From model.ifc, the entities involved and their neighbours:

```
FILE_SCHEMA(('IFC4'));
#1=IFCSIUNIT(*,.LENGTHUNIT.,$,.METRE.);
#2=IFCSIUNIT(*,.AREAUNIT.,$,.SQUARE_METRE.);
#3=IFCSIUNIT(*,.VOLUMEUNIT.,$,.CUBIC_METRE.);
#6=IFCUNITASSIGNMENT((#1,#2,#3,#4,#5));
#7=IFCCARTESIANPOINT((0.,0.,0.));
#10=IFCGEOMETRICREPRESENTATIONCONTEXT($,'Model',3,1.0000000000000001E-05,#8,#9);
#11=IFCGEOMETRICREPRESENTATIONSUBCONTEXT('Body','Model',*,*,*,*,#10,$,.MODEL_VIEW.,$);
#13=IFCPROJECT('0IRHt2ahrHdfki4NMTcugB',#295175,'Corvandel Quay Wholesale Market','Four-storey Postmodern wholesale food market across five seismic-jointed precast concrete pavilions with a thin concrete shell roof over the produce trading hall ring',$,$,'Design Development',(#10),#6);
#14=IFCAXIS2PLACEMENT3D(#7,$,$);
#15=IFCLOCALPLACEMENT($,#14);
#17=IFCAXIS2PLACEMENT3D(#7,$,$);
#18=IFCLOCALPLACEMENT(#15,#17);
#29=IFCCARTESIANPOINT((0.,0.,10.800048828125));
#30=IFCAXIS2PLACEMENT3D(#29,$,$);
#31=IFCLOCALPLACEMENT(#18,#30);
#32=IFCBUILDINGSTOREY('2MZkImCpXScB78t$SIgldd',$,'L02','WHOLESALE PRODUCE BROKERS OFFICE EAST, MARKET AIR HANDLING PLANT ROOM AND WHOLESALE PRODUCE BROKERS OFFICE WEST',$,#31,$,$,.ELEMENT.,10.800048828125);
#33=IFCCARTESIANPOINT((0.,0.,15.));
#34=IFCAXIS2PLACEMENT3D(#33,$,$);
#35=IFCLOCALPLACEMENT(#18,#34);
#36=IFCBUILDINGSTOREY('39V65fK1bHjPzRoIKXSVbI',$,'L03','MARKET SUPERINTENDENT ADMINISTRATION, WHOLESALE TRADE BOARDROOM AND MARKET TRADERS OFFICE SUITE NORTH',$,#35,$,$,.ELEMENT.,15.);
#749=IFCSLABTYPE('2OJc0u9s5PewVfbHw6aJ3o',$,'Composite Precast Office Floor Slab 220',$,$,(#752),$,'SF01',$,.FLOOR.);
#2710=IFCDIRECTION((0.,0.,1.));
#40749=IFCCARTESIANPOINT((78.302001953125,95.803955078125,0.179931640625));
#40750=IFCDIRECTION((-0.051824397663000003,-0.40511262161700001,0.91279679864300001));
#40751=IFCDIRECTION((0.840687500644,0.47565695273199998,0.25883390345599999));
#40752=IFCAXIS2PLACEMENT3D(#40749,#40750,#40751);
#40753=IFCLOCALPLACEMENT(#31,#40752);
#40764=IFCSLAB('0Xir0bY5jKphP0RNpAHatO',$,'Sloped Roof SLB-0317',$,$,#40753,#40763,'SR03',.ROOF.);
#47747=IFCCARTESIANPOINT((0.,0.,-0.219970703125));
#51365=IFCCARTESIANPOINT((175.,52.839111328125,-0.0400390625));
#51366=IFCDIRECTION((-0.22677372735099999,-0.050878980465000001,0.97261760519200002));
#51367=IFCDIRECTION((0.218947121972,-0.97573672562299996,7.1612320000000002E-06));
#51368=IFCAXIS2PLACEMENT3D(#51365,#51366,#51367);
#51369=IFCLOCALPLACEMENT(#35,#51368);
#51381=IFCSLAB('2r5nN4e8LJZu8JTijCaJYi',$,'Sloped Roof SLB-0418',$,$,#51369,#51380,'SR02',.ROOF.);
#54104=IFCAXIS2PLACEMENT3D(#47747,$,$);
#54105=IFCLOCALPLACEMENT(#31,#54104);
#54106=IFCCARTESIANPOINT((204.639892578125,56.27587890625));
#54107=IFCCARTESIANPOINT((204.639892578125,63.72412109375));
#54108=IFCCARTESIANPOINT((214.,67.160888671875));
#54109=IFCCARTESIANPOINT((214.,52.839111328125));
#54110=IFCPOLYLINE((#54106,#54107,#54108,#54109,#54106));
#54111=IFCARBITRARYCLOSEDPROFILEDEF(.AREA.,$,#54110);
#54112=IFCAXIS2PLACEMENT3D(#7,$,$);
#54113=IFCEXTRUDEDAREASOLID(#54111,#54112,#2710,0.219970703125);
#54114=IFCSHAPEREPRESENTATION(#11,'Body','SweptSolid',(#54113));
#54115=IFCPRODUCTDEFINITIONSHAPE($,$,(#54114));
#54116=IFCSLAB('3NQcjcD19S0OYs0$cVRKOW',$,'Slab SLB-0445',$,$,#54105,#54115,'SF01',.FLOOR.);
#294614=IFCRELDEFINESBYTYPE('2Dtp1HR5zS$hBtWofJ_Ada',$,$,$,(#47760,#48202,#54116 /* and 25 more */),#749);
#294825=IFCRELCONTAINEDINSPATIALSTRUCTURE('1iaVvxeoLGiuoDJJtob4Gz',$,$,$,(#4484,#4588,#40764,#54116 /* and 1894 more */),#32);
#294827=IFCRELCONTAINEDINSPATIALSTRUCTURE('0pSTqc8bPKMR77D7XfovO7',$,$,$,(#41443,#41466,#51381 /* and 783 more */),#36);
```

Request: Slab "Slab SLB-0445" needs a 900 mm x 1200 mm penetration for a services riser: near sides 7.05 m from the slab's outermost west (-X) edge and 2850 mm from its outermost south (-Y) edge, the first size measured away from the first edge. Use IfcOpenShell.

```python
import numpy as np
import ifcopenshell
import ifcopenshell.api.feature
import ifcopenshell.api.geometry
import ifcopenshell.api.root
import ifcopenshell.geom
import ifcopenshell.util.placement
import ifcopenshell.util.representation
import ifcopenshell.util.shape
import ifcopenshell.util.unit

model = ifcopenshell.open("model.ifc")
unit_scale = ifcopenshell.util.unit.calculate_unit_scale(model)
settings = ifcopenshell.geom.settings()


def volume(element):
    """Net volume in cubic metres, openings subtracted."""
    shape = ifcopenshell.geom.create_shape(settings, element)
    return ifcopenshell.util.shape.get_volume(shape.geometry)


slab = model.by_id(54116)
before = volume(slab)

# Extent in the slab's own axes, in metres. The edges named are its -X and -Y sides.
slab_shape = ifcopenshell.geom.create_shape(settings, slab)
vertices = ifcopenshell.util.shape.get_vertices(slab_shape.geometry)
x_min, y_min, bottom = vertices.min(axis=0)
top = vertices[:, 2].max()

opening = ifcopenshell.api.root.create_entity(model, ifc_class="IfcOpeningElement", name="Services riser opening", predefined_type="OPENING")
context = ifcopenshell.util.representation.get_context(model, "Model", "Body", "MODEL_VIEW")
width, depth = 0.9, 1.2
outline = [(0.0, 0.0), (width, 0.0), (width, depth), (0.0, depth), (0.0, 0.0)]
# Overshoot both faces by 50 mm so the cut is clean.
shape = ifcopenshell.api.geometry.add_slab_representation(
    model, context=context, depth=top - bottom + 0.1, polyline=outline
)
ifcopenshell.api.geometry.assign_representation(model, product=opening, representation=shape)

matrix = ifcopenshell.util.placement.get_local_placement(slab.ObjectPlacement)
matrix[:, 3] = matrix @ np.append(np.array([x_min + 7.05, y_min + 2.85, bottom - 0.05]) / unit_scale, 1.0)
ifcopenshell.api.geometry.edit_object_placement(model, product=opening, matrix=matrix, is_si=False)
ifcopenshell.api.feature.add_feature(model, feature=opening, element=slab)

after = volume(slab)

print(f"slab volume {before:.3f} -> {after:.3f} m3")

model.write("model-out.ifc")
```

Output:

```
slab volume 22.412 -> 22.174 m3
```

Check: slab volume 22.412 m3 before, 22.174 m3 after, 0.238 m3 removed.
